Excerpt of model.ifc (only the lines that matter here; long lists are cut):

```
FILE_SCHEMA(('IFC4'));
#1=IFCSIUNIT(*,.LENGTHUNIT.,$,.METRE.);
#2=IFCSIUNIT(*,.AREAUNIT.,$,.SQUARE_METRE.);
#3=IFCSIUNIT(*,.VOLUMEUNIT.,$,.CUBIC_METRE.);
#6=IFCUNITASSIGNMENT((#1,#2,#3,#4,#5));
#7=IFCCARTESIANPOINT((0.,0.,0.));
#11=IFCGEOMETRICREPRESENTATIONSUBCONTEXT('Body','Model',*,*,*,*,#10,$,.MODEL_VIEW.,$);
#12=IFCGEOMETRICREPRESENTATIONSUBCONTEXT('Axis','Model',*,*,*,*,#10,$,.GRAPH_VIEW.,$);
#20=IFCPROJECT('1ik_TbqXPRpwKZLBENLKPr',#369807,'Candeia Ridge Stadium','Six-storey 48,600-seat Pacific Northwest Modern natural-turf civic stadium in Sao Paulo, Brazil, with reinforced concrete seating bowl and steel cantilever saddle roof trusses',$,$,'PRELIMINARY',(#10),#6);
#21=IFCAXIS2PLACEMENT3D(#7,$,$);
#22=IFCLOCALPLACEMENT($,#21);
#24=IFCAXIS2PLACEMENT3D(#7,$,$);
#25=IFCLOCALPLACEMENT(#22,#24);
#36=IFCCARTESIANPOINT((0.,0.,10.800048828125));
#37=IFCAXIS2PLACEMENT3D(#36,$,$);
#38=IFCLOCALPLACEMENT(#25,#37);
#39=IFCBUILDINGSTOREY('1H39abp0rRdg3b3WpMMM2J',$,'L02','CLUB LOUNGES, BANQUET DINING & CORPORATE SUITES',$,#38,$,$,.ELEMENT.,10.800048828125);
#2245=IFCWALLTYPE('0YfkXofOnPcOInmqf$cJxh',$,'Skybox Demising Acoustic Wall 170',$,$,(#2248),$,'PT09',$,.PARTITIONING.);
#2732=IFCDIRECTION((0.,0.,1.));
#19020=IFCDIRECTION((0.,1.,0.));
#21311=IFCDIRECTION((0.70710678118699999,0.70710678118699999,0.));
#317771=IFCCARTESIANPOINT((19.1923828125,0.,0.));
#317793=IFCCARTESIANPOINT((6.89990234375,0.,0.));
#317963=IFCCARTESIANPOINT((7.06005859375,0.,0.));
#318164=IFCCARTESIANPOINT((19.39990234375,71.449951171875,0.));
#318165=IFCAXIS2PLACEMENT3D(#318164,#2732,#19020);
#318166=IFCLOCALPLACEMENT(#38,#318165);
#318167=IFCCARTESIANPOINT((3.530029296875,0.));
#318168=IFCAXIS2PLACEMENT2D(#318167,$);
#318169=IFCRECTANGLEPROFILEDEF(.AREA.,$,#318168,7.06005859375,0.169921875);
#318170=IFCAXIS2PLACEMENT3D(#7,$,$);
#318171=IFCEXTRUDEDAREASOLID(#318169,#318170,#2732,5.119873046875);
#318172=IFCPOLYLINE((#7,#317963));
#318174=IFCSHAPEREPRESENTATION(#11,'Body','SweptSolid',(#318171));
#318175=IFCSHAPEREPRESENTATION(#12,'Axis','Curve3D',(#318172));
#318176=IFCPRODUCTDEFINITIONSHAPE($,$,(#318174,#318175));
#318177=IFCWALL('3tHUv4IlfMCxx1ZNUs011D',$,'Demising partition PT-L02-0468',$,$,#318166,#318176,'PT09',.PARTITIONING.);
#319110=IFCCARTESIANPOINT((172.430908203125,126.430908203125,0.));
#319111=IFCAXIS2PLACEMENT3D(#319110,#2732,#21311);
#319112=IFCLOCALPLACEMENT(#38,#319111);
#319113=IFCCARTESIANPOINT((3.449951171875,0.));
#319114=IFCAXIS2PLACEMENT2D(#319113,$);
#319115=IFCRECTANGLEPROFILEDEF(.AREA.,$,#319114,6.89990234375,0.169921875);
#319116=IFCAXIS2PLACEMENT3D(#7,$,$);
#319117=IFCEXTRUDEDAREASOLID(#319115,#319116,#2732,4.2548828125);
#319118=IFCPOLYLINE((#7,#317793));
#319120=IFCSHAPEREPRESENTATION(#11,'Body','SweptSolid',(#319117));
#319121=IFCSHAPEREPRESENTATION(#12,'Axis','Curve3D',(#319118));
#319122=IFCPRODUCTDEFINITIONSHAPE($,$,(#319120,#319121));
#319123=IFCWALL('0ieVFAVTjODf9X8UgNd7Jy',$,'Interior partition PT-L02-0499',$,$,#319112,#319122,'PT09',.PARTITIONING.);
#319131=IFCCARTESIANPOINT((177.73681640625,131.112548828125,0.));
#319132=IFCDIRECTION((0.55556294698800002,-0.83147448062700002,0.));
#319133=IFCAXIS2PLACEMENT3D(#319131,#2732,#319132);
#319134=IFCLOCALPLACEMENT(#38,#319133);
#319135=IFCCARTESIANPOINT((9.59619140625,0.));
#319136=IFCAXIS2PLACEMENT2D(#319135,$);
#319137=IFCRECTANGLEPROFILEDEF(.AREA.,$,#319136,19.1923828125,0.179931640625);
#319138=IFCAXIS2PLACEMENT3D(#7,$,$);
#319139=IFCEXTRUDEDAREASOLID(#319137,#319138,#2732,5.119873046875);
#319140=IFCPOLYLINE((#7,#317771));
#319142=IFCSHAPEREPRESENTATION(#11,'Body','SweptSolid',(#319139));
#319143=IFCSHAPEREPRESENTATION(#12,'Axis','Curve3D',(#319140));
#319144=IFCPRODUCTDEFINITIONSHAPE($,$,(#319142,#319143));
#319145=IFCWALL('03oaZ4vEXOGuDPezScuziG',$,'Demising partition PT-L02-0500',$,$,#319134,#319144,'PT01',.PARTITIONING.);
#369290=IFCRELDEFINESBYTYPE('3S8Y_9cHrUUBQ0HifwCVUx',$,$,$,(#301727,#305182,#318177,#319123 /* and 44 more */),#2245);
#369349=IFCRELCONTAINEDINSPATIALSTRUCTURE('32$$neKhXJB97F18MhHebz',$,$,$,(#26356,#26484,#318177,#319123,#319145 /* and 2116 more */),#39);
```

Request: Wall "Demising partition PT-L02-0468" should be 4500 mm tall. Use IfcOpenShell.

```python
import ifcopenshell
import ifcopenshell.geom
import ifcopenshell.util.representation
import ifcopenshell.util.shape
import ifcopenshell.util.unit

model = ifcopenshell.open("model.ifc")
unit_scale = ifcopenshell.util.unit.calculate_unit_scale(model)
settings = ifcopenshell.geom.settings()


def volume(element):
    """Net volume in cubic metres, openings subtracted."""
    shape = ifcopenshell.geom.create_shape(settings, element)
    return ifcopenshell.util.shape.get_volume(shape.geometry)


wall = model.by_guid("3tHUv4IlfMCxx1ZNUs011D")
before = volume(wall)

body = ifcopenshell.util.representation.get_representation(wall, "Model", "Body")
solid = body.Items[0]
old_height = solid.Depth
solid.Depth = 4.5 / unit_scale
after = volume(wall)

print(f"height {old_height:g} -> {solid.Depth:g}, volume {before:.3f} -> {after:.3f} m3")

model.write("model_edited.ifc")
```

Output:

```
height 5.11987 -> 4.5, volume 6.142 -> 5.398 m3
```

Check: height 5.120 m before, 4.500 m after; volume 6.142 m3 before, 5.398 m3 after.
